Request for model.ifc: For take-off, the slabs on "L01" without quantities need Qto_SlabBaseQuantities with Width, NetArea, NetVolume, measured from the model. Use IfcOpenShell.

First a look at what the model holds.

```python
import ifcopenshell
import ifcopenshell.util.element
import ifcopenshell.util.unit

model = ifcopenshell.open("model.ifc")
print(model.schema)
for unit_type in ("LENGTHUNIT", "AREAUNIT", "VOLUMEUNIT"):
    print(unit_type, ifcopenshell.util.unit.calculate_unit_scale(model, unit_type))
storey = next(s for s in model.by_type("IfcBuildingStorey") if s.Name == "L01")
slabs = [e for e in ifcopenshell.util.element.get_decomposition(storey) if e.is_a("IfcSlab")]
for e in sorted(slabs, key=lambda e: e.id()):
    print(e.id(), e.is_a(), e.Name, list(ifcopenshell.util.element.get_psets(e, qtos_only=True)), sep=" | ")
```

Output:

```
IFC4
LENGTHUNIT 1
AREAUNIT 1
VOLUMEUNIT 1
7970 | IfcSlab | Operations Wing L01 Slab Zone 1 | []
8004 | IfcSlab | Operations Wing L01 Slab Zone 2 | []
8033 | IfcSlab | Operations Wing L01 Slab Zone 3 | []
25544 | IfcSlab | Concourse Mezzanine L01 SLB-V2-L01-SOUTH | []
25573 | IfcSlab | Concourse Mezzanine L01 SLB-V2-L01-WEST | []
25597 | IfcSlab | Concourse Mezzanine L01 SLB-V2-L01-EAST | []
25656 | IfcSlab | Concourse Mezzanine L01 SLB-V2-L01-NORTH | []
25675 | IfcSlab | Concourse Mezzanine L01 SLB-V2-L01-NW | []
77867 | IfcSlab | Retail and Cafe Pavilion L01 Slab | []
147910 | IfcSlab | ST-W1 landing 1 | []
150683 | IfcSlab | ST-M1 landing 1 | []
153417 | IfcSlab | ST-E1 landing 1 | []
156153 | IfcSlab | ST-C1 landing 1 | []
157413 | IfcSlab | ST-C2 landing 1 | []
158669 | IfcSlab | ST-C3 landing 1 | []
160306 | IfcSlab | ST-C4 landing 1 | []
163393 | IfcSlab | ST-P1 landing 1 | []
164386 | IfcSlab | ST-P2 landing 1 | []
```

```python
import ifcopenshell
import ifcopenshell.api.pset
import ifcopenshell.geom
import ifcopenshell.util.element
import ifcopenshell.util.shape
import ifcopenshell.util.unit

model = ifcopenshell.open("model.ifc")
unit_scale = ifcopenshell.util.unit.calculate_unit_scale(model)
area_scale = ifcopenshell.util.unit.calculate_unit_scale(model, "AREAUNIT")
volume_scale = ifcopenshell.util.unit.calculate_unit_scale(model, "VOLUMEUNIT")
settings = ifcopenshell.geom.settings()

storey = next(s for s in model.by_type("IfcBuildingStorey") if s.Name == "L01")
slabs = [e for e in ifcopenshell.util.element.get_decomposition(storey) if e.is_a("IfcSlab")]

for e in sorted(slabs, key=lambda e: e.id()):
    if ifcopenshell.util.element.get_psets(e, qtos_only=True, should_inherit=False):
        continue
    # Geometry comes back in metres, in the element's own axes.
    shape = ifcopenshell.geom.create_shape(settings, e)
    values = {
        "Width": ifcopenshell.util.shape.get_z(shape.geometry) / unit_scale,
        "NetArea": ifcopenshell.util.shape.get_footprint_area(shape.geometry) / area_scale,
        "NetVolume": ifcopenshell.util.shape.get_volume(shape.geometry) / volume_scale,
    }
    qto = ifcopenshell.api.pset.add_qto(model, product=e, name="Qto_SlabBaseQuantities")
    ifcopenshell.api.pset.edit_qto(model, qto=qto, properties=values)
    print(e.id(), {k: round(v, 3) for k, v in values.items()})

model.write("model-out.ifc")
```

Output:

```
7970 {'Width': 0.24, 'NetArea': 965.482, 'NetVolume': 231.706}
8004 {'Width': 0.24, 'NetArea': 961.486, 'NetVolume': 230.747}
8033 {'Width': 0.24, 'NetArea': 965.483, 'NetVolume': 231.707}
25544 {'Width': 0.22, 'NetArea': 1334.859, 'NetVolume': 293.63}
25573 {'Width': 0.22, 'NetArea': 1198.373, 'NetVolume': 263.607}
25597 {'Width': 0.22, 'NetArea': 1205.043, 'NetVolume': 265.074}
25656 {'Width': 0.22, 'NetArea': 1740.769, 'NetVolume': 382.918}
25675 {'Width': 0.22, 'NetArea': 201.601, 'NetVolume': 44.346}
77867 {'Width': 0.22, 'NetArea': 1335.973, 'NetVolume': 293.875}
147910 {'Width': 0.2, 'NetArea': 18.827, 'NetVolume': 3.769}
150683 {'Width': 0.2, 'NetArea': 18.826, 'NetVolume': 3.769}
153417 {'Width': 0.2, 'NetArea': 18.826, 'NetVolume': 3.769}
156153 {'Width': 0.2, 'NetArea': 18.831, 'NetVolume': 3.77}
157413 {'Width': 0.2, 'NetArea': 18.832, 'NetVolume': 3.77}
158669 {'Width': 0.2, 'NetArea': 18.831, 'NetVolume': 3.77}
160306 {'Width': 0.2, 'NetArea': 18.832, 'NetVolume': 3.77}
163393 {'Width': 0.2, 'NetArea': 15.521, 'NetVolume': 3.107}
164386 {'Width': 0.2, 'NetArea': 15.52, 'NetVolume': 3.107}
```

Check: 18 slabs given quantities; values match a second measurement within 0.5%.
